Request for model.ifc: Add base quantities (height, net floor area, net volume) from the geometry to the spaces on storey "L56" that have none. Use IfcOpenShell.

First a look at what the model holds.

```python
import ifcopenshell
import ifcopenshell.util.element
import ifcopenshell.util.unit

model = ifcopenshell.open("model.ifc")
print(model.schema)
for unit_type in ("LENGTHUNIT", "AREAUNIT", "VOLUMEUNIT"):
    print(unit_type, ifcopenshell.util.unit.calculate_unit_scale(model, unit_type))
storey = next(s for s in model.by_type("IfcBuildingStorey") if s.Name == "L56")
spaces = [e for e in ifcopenshell.util.element.get_decomposition(storey) if e.is_a("IfcSpace")]
for e in sorted(spaces, key=lambda e: e.id()):
    print(e.id(), e.is_a(), e.Name, list(ifcopenshell.util.element.get_psets(e, qtos_only=True)), sep=" | ")
```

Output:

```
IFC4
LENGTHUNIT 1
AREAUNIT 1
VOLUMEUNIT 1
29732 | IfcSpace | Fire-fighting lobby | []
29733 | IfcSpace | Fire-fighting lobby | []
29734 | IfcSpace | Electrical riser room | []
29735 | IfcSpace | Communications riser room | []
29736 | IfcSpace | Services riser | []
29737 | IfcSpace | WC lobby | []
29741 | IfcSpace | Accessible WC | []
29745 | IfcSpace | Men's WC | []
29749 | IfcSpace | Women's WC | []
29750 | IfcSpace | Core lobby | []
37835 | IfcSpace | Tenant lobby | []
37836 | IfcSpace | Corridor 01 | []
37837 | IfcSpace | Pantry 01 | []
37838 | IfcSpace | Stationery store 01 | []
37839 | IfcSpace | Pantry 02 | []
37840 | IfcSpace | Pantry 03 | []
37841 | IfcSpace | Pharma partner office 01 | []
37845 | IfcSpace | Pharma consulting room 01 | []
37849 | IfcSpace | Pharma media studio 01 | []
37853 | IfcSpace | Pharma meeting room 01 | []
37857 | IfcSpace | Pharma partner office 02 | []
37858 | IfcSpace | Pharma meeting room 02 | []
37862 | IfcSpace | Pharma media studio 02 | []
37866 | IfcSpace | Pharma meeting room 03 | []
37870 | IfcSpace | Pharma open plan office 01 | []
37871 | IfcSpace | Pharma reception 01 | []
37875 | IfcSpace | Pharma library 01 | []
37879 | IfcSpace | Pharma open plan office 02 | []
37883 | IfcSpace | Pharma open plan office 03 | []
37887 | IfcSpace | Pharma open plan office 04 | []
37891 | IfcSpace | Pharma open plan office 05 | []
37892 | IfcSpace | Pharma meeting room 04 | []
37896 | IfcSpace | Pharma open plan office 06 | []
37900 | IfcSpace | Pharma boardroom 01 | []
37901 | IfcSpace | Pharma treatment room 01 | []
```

```python
import ifcopenshell
import ifcopenshell.api.pset
import ifcopenshell.geom
import ifcopenshell.util.element
import ifcopenshell.util.shape
import ifcopenshell.util.unit

model = ifcopenshell.open("model.ifc")
unit_scale = ifcopenshell.util.unit.calculate_unit_scale(model)
area_scale = ifcopenshell.util.unit.calculate_unit_scale(model, "AREAUNIT")
volume_scale = ifcopenshell.util.unit.calculate_unit_scale(model, "VOLUMEUNIT")
settings = ifcopenshell.geom.settings()

storey = next(s for s in model.by_type("IfcBuildingStorey") if s.Name == "L56")
spaces = [e for e in ifcopenshell.util.element.get_decomposition(storey) if e.is_a("IfcSpace")]

for e in sorted(spaces, key=lambda e: e.id()):
    if ifcopenshell.util.element.get_psets(e, qtos_only=True, should_inherit=False):
        continue
    # Geometry comes back in metres, in the element's own axes.
    shape = ifcopenshell.geom.create_shape(settings, e)
    values = {
        "Height": ifcopenshell.util.shape.get_z(shape.geometry) / unit_scale,
        "NetFloorArea": ifcopenshell.util.shape.get_footprint_area(shape.geometry) / area_scale,
        "NetVolume": ifcopenshell.util.shape.get_volume(shape.geometry) / volume_scale,
    }
    qto = ifcopenshell.api.pset.add_qto(model, product=e, name="Qto_SpaceBaseQuantities")
    ifcopenshell.api.pset.edit_qto(model, qto=qto, properties=values)
    print(e.id(), {k: round(v, 3) for k, v in values.items()})

model.write("model_edited.ifc")
```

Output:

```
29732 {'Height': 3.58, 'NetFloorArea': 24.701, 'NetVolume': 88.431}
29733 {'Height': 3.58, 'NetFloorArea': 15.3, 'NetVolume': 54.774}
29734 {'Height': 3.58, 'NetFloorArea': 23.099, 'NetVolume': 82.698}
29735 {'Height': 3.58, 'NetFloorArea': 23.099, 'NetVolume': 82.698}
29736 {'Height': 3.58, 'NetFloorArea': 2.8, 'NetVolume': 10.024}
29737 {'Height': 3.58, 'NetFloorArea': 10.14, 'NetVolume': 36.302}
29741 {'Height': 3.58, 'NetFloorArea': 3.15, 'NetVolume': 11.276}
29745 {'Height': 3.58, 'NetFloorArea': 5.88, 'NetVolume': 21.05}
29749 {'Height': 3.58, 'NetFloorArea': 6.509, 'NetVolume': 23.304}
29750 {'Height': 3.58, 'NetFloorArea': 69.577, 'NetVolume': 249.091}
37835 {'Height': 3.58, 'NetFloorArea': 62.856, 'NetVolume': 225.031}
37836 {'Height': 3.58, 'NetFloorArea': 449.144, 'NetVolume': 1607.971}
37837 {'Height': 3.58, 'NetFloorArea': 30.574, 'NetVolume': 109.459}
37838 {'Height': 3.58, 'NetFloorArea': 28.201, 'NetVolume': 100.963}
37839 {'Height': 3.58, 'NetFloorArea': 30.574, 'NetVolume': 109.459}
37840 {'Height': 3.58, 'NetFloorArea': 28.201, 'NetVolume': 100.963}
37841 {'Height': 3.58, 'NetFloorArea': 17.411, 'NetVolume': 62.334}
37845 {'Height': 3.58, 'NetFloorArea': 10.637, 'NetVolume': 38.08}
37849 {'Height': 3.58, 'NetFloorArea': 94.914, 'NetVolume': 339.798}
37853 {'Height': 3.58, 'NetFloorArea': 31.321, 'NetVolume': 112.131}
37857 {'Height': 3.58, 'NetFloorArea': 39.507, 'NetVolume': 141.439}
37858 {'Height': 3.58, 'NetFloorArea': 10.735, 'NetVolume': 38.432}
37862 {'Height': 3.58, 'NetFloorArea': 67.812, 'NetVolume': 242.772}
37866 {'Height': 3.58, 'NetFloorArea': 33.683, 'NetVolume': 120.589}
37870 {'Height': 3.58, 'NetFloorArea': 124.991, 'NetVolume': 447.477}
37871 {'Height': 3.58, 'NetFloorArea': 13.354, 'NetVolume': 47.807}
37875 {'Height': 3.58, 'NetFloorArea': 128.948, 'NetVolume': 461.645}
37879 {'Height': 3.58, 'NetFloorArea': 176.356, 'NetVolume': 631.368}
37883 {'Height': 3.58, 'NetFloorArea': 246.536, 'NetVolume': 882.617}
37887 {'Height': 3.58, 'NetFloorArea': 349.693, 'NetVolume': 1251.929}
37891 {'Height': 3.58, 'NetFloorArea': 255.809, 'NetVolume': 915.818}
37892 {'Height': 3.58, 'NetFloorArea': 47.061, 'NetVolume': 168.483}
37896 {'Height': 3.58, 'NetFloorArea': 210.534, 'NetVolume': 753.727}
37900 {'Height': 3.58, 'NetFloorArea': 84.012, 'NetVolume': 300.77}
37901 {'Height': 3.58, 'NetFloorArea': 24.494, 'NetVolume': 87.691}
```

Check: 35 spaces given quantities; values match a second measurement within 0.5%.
